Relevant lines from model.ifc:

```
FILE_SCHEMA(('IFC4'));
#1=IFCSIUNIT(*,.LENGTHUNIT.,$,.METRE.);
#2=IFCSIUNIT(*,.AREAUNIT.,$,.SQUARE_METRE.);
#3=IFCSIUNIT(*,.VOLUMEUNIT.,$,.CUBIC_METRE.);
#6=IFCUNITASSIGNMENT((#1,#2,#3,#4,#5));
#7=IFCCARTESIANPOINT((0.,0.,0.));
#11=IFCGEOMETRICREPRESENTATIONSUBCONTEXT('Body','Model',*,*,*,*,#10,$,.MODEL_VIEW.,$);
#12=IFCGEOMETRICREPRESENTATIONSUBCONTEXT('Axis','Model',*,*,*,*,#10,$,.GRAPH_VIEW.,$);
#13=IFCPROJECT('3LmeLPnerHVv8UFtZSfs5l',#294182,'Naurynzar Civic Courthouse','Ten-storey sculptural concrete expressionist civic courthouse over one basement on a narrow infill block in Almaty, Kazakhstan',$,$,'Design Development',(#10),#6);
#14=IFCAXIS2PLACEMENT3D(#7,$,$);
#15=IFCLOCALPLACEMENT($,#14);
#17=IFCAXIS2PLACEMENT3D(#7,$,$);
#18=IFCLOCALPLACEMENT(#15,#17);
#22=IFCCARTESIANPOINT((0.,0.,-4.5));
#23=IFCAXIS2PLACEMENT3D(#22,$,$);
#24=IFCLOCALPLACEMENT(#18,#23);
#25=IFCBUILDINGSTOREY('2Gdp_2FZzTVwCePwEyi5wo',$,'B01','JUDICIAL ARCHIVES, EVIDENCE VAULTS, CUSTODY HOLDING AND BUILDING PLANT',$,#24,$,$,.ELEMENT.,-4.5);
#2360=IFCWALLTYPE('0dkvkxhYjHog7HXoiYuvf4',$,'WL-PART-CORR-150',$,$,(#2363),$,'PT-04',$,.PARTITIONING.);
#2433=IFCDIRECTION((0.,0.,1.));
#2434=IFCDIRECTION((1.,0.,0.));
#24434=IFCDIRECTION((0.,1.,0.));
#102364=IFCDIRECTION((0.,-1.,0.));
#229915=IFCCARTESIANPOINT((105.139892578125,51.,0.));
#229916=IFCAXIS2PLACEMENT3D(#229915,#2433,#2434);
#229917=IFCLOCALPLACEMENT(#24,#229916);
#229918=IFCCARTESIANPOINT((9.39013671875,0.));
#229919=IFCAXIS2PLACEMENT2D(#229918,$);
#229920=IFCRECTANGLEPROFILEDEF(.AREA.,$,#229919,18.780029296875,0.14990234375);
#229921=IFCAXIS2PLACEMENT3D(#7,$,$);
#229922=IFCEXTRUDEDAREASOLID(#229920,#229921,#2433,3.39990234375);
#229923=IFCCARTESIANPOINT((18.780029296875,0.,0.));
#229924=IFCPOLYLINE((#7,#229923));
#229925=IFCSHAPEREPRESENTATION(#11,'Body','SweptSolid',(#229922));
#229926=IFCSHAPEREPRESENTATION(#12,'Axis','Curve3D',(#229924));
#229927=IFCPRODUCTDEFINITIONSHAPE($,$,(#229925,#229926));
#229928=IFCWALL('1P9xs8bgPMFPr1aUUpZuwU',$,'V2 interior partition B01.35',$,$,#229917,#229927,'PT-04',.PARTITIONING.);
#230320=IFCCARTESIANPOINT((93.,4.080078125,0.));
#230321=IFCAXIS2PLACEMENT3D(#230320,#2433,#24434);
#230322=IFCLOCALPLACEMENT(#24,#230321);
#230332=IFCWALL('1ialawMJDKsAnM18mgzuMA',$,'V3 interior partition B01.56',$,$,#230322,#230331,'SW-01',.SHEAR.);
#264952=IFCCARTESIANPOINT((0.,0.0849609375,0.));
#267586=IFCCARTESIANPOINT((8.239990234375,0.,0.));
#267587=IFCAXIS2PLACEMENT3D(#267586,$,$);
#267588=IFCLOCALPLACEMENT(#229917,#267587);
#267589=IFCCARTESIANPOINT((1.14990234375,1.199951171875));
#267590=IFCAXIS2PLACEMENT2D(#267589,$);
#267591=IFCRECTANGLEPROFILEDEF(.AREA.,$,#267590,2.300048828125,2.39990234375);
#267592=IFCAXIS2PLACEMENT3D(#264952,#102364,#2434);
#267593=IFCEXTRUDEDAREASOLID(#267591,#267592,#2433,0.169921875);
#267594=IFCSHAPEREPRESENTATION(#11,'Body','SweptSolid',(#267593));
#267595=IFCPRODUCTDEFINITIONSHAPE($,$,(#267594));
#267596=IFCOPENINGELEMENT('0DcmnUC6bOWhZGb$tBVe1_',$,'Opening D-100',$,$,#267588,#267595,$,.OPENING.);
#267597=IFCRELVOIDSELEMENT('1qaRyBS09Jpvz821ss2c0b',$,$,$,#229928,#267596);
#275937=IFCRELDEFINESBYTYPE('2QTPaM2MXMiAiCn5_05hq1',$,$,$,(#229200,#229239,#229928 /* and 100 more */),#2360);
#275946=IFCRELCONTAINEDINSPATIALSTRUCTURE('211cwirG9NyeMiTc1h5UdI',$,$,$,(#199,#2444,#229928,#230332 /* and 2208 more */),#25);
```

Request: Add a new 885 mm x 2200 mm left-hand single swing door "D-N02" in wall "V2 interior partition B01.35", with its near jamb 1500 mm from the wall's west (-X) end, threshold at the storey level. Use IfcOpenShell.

```python
import numpy as np
import ifcopenshell
import ifcopenshell.api.feature
import ifcopenshell.api.geometry
import ifcopenshell.api.root
import ifcopenshell.api.spatial
import ifcopenshell.geom
import ifcopenshell.util.element
import ifcopenshell.util.placement
import ifcopenshell.util.representation
import ifcopenshell.util.shape
import ifcopenshell.util.unit

model = ifcopenshell.open("model.ifc")
unit_scale = ifcopenshell.util.unit.calculate_unit_scale(model)
settings = ifcopenshell.geom.settings()


def volume(element):
    """Net volume in cubic metres, openings subtracted."""
    shape = ifcopenshell.geom.create_shape(settings, element)
    return ifcopenshell.util.shape.get_volume(shape.geometry)


wall = model.by_id(229928)
storey = ifcopenshell.util.element.get_container(wall, ifc_class="IfcBuildingStorey")
context = ifcopenshell.util.representation.get_context(model, "Model", "Body", "MODEL_VIEW")
before = volume(wall)

width, height, from_end, sill = 0.885, 2.2, 1.5, 0.0  # metres

# The wall runs along its own X axis, and the end named is its -X end.
wall_shape = ifcopenshell.geom.create_shape(settings, wall)
x, y, z = ifcopenshell.util.shape.get_vertices(wall_shape.geometry).T
start = x.min() + from_end
face, thickness = float(y.min()), float(y.max() - y.min())
wall_matrix = ifcopenshell.util.placement.get_local_placement(wall.ObjectPlacement)
level = ifcopenshell.util.placement.get_local_placement(storey.ObjectPlacement)[2, 3]


def in_wall(x, y):
    """Placement at x, y metres in the wall's axes, at sill height."""
    matrix = wall_matrix.copy()
    matrix[:, 3] = wall_matrix @ np.array([x / unit_scale, y / unit_scale, 0.0, 1.0])
    matrix[2, 3] = level + sill / unit_scale
    return matrix


# Opening: a box that overshoots both wall faces by 50 mm.
opening = ifcopenshell.api.root.create_entity(model, ifc_class="IfcOpeningElement", predefined_type="OPENING")
box = ifcopenshell.api.geometry.add_wall_representation(
    model, context=context, length=width, height=height, thickness=thickness + 0.1
)
ifcopenshell.api.geometry.assign_representation(model, product=opening, representation=box)
ifcopenshell.api.geometry.edit_object_placement(model, product=opening, matrix=in_wall(start, face - 0.05), is_si=False)
ifcopenshell.api.feature.add_feature(model, feature=opening, element=wall)

door = ifcopenshell.api.root.create_entity(model, ifc_class="IfcDoor", name="D-N02", predefined_type="DOOR")
door.OverallWidth, door.OverallHeight = width / unit_scale, height / unit_scale
door.OperationType = "SINGLE_SWING_LEFT"
body = ifcopenshell.api.geometry.add_door_representation(
    model,
    context=context,
    overall_width=door.OverallWidth,
    overall_height=door.OverallHeight,
    operation_type="SINGLE_SWING_LEFT",
    lining_properties={"LiningDepth": thickness / unit_scale, "ThresholdDepth": thickness / unit_scale},
)
ifcopenshell.api.geometry.assign_representation(model, product=door, representation=body)
ifcopenshell.api.spatial.assign_container(model, products=[door], relating_structure=storey)
ifcopenshell.api.feature.add_filling(model, opening=opening, element=door)

# The lining spans the wall, so the door starts at the wall face.
ifcopenshell.api.geometry.edit_object_placement(model, product=door, matrix=in_wall(start, face), is_si=False)

after = volume(wall)

print(f"wall volume {before:.3f} -> {after:.3f} m3")

model.write("model_v2.ifc")
```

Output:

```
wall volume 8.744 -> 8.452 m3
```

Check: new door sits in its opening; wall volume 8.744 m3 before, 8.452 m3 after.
